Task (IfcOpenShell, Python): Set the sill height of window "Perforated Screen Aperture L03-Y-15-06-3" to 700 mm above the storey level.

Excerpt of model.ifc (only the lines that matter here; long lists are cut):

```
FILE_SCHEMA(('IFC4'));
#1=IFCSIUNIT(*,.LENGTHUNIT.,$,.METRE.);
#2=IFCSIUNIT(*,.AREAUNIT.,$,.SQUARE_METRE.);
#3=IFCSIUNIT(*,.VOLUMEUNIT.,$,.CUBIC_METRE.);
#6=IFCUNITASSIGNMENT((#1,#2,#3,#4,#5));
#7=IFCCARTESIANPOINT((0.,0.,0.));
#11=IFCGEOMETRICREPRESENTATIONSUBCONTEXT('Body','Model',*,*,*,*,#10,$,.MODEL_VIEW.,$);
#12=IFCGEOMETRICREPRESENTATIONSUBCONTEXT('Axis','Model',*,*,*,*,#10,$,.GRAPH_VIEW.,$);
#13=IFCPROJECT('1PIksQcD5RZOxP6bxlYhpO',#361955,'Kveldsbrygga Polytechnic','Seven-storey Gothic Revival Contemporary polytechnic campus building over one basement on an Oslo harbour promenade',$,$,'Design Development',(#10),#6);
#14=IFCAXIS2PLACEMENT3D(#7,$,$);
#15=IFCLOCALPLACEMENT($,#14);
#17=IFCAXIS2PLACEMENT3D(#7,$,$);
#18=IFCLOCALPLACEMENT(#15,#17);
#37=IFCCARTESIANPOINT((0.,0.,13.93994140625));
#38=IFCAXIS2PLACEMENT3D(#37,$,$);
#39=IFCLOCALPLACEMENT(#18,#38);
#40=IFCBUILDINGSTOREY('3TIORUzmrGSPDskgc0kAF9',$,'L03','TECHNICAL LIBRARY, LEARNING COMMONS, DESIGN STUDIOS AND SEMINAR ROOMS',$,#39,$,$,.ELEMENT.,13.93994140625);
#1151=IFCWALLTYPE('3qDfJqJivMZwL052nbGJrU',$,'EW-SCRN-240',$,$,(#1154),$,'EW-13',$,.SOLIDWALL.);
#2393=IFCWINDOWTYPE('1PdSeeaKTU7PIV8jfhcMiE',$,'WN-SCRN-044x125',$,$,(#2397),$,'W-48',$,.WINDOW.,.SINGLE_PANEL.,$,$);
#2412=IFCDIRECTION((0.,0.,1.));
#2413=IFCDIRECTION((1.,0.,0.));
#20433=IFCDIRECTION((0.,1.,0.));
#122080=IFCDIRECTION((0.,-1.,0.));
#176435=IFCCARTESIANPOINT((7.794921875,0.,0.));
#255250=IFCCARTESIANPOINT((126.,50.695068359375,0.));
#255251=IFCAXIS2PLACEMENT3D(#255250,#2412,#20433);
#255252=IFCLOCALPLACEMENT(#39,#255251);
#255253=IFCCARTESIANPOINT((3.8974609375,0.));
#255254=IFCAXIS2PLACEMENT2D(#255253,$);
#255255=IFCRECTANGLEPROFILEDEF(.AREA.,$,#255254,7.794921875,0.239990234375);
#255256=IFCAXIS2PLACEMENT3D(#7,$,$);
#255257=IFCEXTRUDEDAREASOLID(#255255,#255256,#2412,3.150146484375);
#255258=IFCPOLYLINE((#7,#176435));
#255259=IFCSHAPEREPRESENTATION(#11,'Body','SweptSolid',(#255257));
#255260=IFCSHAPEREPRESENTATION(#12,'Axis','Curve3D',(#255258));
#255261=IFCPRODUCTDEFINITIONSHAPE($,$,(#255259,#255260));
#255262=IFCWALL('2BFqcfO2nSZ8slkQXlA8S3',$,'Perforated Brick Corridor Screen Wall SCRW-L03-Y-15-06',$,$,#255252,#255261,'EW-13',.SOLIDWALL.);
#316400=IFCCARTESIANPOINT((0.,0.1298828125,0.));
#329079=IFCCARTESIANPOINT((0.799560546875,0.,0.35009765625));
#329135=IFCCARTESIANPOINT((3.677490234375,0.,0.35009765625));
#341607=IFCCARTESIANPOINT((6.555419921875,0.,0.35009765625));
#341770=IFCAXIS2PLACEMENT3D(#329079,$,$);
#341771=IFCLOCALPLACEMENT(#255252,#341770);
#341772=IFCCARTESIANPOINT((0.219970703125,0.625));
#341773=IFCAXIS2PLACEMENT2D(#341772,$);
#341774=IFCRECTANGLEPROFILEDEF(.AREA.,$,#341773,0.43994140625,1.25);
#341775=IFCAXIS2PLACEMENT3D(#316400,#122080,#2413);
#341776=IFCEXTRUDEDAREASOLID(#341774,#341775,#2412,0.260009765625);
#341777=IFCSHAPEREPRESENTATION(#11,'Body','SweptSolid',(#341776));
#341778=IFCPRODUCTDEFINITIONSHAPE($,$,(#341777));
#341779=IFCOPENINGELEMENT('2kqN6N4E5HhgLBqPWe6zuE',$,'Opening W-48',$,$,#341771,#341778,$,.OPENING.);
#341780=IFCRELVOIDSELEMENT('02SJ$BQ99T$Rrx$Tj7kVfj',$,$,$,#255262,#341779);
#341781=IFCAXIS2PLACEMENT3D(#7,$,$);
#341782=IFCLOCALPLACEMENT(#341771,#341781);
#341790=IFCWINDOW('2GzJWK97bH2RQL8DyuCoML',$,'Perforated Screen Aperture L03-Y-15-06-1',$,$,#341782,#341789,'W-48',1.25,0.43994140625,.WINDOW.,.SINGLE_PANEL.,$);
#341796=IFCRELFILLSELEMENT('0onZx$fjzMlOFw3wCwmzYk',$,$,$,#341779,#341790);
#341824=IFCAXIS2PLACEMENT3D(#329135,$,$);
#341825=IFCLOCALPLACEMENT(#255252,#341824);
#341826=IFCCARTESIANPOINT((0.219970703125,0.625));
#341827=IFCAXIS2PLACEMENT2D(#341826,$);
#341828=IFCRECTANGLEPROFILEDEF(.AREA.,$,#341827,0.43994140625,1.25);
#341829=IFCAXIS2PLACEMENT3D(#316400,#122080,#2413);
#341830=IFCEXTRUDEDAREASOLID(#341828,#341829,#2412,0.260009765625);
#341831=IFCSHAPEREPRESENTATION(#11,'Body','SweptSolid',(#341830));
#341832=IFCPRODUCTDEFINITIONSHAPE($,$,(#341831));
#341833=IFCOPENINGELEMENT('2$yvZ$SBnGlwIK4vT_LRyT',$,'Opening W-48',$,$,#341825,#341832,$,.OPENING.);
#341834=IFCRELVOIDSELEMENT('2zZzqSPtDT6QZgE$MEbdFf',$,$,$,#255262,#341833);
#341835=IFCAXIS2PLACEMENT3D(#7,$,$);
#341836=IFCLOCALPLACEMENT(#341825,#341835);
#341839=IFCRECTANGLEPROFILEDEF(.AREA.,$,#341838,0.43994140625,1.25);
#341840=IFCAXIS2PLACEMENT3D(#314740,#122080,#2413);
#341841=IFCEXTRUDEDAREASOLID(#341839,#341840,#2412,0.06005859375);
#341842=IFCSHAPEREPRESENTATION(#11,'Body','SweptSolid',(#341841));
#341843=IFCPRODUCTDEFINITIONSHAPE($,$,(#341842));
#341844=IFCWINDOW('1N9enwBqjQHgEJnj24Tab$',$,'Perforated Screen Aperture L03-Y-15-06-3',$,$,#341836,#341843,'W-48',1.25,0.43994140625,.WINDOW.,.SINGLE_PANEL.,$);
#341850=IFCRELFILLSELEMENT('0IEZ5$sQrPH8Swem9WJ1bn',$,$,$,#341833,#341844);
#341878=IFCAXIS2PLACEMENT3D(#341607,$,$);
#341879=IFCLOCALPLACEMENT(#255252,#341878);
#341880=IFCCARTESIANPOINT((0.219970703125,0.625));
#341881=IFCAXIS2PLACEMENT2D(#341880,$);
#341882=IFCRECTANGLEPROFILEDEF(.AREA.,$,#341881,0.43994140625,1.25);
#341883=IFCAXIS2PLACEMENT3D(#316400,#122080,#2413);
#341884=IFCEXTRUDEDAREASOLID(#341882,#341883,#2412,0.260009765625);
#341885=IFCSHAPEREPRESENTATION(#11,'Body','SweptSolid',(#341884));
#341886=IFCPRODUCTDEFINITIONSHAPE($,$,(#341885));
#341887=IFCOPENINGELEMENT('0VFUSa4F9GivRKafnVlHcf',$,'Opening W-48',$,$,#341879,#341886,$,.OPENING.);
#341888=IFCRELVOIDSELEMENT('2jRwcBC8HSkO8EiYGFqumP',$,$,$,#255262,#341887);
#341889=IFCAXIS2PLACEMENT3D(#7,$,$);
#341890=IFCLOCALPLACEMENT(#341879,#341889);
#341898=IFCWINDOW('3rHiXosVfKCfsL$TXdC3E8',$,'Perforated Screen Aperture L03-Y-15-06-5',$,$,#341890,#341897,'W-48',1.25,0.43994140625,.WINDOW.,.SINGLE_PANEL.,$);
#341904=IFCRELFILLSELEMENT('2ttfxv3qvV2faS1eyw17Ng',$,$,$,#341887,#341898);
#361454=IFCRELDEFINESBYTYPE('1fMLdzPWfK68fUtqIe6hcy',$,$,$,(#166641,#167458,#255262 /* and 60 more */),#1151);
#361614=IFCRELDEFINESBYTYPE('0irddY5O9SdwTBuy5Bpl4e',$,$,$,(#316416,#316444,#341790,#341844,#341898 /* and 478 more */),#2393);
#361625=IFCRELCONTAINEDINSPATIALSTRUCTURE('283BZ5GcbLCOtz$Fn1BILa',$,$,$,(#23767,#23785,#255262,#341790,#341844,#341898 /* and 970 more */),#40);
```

```python
import numpy as np
import ifcopenshell
import ifcopenshell.api.geometry
import ifcopenshell.geom
import ifcopenshell.util.element
import ifcopenshell.util.placement
import ifcopenshell.util.shape
import ifcopenshell.util.unit

model = ifcopenshell.open("model.ifc")
unit_scale = ifcopenshell.util.unit.calculate_unit_scale(model)

window = model.by_guid("1N9enwBqjQHgEJnj24Tab$")
opening = window.FillsVoids[0].RelatingOpeningElement
storey = ifcopenshell.util.element.get_container(window, ifc_class="IfcBuildingStorey")
level = ifcopenshell.util.placement.get_local_placement(storey.ObjectPlacement)[2, 3]

# The opening's origin need not be at the sill, so measure its lowest point.
shape = ifcopenshell.geom.create_shape(ifcopenshell.geom.settings(), opening)
bottom = ifcopenshell.util.shape.get_shape_bottom_elevation(shape, shape.geometry) / unit_scale
dz = level + 0.7 - bottom

shift = np.array([0.0, 0.0, dz])
# The window is placed relative to its opening, so it follows when the opening moves.
matrix = ifcopenshell.util.placement.get_local_placement(opening.ObjectPlacement)
matrix[:3, 3] += shift
ifcopenshell.api.geometry.edit_object_placement(
    model, product=opening, matrix=matrix, is_si=False, should_transform_children=True
)

print(f"moved by {dz * unit_scale:+.3f} m")

model.write("model_v2.ifc")
```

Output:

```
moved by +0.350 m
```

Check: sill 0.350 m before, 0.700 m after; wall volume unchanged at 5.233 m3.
